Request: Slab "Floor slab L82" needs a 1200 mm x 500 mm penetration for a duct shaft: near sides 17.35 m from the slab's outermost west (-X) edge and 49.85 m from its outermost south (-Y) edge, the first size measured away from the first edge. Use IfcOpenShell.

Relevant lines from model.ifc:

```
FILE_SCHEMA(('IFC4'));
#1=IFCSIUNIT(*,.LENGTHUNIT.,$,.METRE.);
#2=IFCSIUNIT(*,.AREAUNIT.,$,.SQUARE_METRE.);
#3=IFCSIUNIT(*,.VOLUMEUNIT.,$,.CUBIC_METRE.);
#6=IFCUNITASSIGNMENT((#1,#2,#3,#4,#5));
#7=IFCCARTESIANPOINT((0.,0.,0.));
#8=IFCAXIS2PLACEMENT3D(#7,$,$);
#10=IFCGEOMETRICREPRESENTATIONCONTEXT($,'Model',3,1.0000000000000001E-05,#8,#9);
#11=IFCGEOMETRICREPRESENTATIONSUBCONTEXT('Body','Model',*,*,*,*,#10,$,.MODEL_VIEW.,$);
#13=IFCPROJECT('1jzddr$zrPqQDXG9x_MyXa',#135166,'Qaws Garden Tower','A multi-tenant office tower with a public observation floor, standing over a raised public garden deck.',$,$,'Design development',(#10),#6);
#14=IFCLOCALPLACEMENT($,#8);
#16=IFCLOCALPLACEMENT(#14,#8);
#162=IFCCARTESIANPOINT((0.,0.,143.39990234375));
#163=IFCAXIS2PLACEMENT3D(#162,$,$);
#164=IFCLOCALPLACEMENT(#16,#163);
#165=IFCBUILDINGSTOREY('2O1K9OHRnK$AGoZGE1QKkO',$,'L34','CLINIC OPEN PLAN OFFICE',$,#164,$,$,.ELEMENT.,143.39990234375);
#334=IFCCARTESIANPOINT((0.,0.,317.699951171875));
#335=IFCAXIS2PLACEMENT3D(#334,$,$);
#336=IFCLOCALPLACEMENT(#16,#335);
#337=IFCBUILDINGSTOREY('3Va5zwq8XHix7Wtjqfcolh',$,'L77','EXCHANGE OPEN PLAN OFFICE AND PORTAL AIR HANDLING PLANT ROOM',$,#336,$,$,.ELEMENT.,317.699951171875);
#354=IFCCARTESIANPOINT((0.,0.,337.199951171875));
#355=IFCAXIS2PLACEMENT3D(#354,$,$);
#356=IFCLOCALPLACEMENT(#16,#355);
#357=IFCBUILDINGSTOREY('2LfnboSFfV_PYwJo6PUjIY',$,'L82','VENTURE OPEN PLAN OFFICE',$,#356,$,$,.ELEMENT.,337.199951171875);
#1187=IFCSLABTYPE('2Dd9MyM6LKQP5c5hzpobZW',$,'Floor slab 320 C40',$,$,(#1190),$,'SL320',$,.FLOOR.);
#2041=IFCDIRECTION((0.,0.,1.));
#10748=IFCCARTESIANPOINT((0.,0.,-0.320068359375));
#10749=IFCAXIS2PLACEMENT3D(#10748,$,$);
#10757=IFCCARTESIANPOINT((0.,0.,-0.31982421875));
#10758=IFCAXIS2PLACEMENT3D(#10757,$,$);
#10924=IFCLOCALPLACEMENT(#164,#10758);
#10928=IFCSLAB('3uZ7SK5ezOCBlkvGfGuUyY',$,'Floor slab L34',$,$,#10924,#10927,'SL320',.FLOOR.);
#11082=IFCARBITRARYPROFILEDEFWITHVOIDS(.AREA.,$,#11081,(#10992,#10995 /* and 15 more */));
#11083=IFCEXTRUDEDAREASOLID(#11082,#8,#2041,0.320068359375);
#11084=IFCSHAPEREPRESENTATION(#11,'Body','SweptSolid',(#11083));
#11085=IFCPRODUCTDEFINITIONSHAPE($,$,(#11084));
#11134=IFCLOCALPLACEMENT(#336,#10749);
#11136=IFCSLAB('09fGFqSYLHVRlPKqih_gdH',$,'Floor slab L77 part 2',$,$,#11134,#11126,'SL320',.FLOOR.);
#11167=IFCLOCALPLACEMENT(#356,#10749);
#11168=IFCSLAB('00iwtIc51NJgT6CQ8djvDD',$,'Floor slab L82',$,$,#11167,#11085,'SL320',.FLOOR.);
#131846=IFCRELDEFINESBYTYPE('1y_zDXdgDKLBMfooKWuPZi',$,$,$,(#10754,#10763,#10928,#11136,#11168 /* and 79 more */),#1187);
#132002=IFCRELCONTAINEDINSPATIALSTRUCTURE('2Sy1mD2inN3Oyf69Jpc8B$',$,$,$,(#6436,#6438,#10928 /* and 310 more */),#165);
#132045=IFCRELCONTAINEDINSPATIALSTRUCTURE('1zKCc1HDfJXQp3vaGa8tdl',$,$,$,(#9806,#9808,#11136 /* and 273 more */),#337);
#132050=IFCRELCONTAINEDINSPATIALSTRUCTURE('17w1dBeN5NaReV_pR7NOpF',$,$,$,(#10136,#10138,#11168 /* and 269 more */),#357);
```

```python
import numpy as np
import ifcopenshell
import ifcopenshell.api.feature
import ifcopenshell.api.geometry
import ifcopenshell.api.root
import ifcopenshell.geom
import ifcopenshell.util.placement
import ifcopenshell.util.representation
import ifcopenshell.util.shape
import ifcopenshell.util.unit

model = ifcopenshell.open("model.ifc")
unit_scale = ifcopenshell.util.unit.calculate_unit_scale(model)
settings = ifcopenshell.geom.settings()


def volume(element):
    """Net volume in cubic metres, openings subtracted."""
    shape = ifcopenshell.geom.create_shape(settings, element)
    return ifcopenshell.util.shape.get_volume(shape.geometry)


slab = model.by_guid("00iwtIc51NJgT6CQ8djvDD")
before = volume(slab)

# Extent in the slab's own axes, in metres. The edges named are its -X and -Y sides.
slab_shape = ifcopenshell.geom.create_shape(settings, slab)
vertices = ifcopenshell.util.shape.get_vertices(slab_shape.geometry)
x_min, y_min, bottom = vertices.min(axis=0)
top = vertices[:, 2].max()

opening = ifcopenshell.api.root.create_entity(model, ifc_class="IfcOpeningElement", name="Duct shaft opening", predefined_type="OPENING")
context = ifcopenshell.util.representation.get_context(model, "Model", "Body", "MODEL_VIEW")
width, depth = 1.2, 0.5
outline = [(0.0, 0.0), (width, 0.0), (width, depth), (0.0, depth), (0.0, 0.0)]
# Overshoot both faces by 50 mm so the cut is clean.
shape = ifcopenshell.api.geometry.add_slab_representation(
    model, context=context, depth=top - bottom + 0.1, polyline=outline
)
ifcopenshell.api.geometry.assign_representation(model, product=opening, representation=shape)

matrix = ifcopenshell.util.placement.get_local_placement(slab.ObjectPlacement)
matrix[:, 3] = matrix @ np.append(np.array([x_min + 17.35, y_min + 49.85, bottom - 0.05]) / unit_scale, 1.0)
ifcopenshell.api.geometry.edit_object_placement(model, product=opening, matrix=matrix, is_si=False)
ifcopenshell.api.feature.add_feature(model, feature=opening, element=slab)

after = volume(slab)

print(f"slab volume {before:.3f} -> {after:.3f} m3")

model.write("model_edited.ifc")
```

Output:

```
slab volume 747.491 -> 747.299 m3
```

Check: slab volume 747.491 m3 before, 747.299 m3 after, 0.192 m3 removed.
